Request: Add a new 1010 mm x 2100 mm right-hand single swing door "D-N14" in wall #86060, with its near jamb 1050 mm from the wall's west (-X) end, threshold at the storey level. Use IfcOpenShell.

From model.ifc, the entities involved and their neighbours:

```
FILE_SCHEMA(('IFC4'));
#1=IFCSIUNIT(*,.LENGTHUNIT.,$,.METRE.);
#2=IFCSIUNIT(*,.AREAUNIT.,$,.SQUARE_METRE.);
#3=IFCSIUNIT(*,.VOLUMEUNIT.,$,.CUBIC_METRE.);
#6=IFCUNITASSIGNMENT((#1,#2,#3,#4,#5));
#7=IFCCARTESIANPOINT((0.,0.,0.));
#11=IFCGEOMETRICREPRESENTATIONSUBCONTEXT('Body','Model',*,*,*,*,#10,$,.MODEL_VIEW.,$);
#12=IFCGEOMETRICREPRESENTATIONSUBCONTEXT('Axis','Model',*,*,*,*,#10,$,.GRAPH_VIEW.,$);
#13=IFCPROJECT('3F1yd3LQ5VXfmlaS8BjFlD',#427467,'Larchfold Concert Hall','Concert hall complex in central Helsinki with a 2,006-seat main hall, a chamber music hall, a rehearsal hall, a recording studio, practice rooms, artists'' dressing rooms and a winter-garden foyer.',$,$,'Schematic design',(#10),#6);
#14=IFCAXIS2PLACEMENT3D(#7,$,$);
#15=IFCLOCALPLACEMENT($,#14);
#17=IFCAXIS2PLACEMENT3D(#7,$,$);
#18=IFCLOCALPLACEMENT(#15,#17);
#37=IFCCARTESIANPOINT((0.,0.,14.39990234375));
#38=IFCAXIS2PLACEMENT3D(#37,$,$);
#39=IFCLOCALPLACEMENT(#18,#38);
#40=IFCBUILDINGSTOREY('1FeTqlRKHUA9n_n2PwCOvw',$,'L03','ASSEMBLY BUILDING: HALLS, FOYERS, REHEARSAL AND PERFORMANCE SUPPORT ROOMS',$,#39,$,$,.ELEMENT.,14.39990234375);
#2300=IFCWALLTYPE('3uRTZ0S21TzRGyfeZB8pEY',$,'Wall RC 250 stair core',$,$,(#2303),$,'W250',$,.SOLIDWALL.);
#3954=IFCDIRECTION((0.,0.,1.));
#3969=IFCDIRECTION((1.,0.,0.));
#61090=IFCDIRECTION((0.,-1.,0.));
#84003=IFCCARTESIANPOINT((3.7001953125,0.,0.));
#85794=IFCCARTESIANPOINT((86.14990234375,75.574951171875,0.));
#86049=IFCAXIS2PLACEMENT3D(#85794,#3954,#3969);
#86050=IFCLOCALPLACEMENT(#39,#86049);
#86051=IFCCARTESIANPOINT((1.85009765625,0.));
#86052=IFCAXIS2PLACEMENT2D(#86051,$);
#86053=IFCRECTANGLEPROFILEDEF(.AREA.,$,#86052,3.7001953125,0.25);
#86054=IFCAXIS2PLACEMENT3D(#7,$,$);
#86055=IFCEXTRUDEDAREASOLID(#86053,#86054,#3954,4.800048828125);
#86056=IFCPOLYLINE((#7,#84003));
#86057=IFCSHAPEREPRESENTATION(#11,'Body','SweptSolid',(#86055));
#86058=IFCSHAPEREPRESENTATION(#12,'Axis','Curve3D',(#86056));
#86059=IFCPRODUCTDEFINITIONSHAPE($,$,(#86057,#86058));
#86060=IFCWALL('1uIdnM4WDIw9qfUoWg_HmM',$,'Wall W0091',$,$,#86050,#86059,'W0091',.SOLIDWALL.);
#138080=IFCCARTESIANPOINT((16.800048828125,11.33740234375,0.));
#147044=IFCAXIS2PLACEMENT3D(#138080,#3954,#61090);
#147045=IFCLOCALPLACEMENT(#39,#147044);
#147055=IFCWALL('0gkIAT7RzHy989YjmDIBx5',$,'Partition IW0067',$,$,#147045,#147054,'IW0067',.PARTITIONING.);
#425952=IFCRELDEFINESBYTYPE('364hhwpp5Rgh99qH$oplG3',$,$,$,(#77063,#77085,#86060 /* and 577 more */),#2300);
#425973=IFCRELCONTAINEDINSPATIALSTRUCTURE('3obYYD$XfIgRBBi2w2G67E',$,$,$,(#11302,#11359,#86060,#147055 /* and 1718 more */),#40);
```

```python
import numpy as np
import ifcopenshell
import ifcopenshell.api.feature
import ifcopenshell.api.geometry
import ifcopenshell.api.root
import ifcopenshell.api.spatial
import ifcopenshell.geom
import ifcopenshell.util.element
import ifcopenshell.util.placement
import ifcopenshell.util.representation
import ifcopenshell.util.shape
import ifcopenshell.util.unit

model = ifcopenshell.open("model.ifc")
unit_scale = ifcopenshell.util.unit.calculate_unit_scale(model)
settings = ifcopenshell.geom.settings()


def volume(element):
    """Net volume in cubic metres, openings subtracted."""
    shape = ifcopenshell.geom.create_shape(settings, element)
    return ifcopenshell.util.shape.get_volume(shape.geometry)


wall = model.by_guid("1uIdnM4WDIw9qfUoWg_HmM")
storey = ifcopenshell.util.element.get_container(wall, ifc_class="IfcBuildingStorey")
context = ifcopenshell.util.representation.get_context(model, "Model", "Body", "MODEL_VIEW")
before = volume(wall)

width, height, from_end, sill = 1.01, 2.1, 1.05, 0.0  # metres

# The wall runs along its own X axis, and the end named is its -X end.
wall_shape = ifcopenshell.geom.create_shape(settings, wall)
x, y, z = ifcopenshell.util.shape.get_vertices(wall_shape.geometry).T
start = x.min() + from_end
face, thickness = float(y.min()), float(y.max() - y.min())
wall_matrix = ifcopenshell.util.placement.get_local_placement(wall.ObjectPlacement)
level = ifcopenshell.util.placement.get_local_placement(storey.ObjectPlacement)[2, 3]


def in_wall(x, y):
    """Placement at x, y metres in the wall's axes, at sill height."""
    matrix = wall_matrix.copy()
    matrix[:, 3] = wall_matrix @ np.array([x / unit_scale, y / unit_scale, 0.0, 1.0])
    matrix[2, 3] = level + sill / unit_scale
    return matrix


# Opening: a box that overshoots both wall faces by 50 mm.
opening = ifcopenshell.api.root.create_entity(model, ifc_class="IfcOpeningElement", predefined_type="OPENING")
box = ifcopenshell.api.geometry.add_wall_representation(
    model, context=context, length=width, height=height, thickness=thickness + 0.1
)
ifcopenshell.api.geometry.assign_representation(model, product=opening, representation=box)
ifcopenshell.api.geometry.edit_object_placement(model, product=opening, matrix=in_wall(start, face - 0.05), is_si=False)
ifcopenshell.api.feature.add_feature(model, feature=opening, element=wall)

door = ifcopenshell.api.root.create_entity(model, ifc_class="IfcDoor", name="D-N14", predefined_type="DOOR")
door.OverallWidth, door.OverallHeight = width / unit_scale, height / unit_scale
door.OperationType = "SINGLE_SWING_RIGHT"
body = ifcopenshell.api.geometry.add_door_representation(
    model,
    context=context,
    overall_width=door.OverallWidth,
    overall_height=door.OverallHeight,
    operation_type="SINGLE_SWING_RIGHT",
    lining_properties={"LiningDepth": thickness / unit_scale, "ThresholdDepth": thickness / unit_scale},
)
ifcopenshell.api.geometry.assign_representation(model, product=door, representation=body)
ifcopenshell.api.spatial.assign_container(model, products=[door], relating_structure=storey)
ifcopenshell.api.feature.add_filling(model, opening=opening, element=door)

# The lining spans the wall, so the door starts at the wall face.
ifcopenshell.api.geometry.edit_object_placement(model, product=door, matrix=in_wall(start, face), is_si=False)

after = volume(wall)

print(f"wall volume {before:.3f} -> {after:.3f} m3")

model.write("model_edited.ifc")
```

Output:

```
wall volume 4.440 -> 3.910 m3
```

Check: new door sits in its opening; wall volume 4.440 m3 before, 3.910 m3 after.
